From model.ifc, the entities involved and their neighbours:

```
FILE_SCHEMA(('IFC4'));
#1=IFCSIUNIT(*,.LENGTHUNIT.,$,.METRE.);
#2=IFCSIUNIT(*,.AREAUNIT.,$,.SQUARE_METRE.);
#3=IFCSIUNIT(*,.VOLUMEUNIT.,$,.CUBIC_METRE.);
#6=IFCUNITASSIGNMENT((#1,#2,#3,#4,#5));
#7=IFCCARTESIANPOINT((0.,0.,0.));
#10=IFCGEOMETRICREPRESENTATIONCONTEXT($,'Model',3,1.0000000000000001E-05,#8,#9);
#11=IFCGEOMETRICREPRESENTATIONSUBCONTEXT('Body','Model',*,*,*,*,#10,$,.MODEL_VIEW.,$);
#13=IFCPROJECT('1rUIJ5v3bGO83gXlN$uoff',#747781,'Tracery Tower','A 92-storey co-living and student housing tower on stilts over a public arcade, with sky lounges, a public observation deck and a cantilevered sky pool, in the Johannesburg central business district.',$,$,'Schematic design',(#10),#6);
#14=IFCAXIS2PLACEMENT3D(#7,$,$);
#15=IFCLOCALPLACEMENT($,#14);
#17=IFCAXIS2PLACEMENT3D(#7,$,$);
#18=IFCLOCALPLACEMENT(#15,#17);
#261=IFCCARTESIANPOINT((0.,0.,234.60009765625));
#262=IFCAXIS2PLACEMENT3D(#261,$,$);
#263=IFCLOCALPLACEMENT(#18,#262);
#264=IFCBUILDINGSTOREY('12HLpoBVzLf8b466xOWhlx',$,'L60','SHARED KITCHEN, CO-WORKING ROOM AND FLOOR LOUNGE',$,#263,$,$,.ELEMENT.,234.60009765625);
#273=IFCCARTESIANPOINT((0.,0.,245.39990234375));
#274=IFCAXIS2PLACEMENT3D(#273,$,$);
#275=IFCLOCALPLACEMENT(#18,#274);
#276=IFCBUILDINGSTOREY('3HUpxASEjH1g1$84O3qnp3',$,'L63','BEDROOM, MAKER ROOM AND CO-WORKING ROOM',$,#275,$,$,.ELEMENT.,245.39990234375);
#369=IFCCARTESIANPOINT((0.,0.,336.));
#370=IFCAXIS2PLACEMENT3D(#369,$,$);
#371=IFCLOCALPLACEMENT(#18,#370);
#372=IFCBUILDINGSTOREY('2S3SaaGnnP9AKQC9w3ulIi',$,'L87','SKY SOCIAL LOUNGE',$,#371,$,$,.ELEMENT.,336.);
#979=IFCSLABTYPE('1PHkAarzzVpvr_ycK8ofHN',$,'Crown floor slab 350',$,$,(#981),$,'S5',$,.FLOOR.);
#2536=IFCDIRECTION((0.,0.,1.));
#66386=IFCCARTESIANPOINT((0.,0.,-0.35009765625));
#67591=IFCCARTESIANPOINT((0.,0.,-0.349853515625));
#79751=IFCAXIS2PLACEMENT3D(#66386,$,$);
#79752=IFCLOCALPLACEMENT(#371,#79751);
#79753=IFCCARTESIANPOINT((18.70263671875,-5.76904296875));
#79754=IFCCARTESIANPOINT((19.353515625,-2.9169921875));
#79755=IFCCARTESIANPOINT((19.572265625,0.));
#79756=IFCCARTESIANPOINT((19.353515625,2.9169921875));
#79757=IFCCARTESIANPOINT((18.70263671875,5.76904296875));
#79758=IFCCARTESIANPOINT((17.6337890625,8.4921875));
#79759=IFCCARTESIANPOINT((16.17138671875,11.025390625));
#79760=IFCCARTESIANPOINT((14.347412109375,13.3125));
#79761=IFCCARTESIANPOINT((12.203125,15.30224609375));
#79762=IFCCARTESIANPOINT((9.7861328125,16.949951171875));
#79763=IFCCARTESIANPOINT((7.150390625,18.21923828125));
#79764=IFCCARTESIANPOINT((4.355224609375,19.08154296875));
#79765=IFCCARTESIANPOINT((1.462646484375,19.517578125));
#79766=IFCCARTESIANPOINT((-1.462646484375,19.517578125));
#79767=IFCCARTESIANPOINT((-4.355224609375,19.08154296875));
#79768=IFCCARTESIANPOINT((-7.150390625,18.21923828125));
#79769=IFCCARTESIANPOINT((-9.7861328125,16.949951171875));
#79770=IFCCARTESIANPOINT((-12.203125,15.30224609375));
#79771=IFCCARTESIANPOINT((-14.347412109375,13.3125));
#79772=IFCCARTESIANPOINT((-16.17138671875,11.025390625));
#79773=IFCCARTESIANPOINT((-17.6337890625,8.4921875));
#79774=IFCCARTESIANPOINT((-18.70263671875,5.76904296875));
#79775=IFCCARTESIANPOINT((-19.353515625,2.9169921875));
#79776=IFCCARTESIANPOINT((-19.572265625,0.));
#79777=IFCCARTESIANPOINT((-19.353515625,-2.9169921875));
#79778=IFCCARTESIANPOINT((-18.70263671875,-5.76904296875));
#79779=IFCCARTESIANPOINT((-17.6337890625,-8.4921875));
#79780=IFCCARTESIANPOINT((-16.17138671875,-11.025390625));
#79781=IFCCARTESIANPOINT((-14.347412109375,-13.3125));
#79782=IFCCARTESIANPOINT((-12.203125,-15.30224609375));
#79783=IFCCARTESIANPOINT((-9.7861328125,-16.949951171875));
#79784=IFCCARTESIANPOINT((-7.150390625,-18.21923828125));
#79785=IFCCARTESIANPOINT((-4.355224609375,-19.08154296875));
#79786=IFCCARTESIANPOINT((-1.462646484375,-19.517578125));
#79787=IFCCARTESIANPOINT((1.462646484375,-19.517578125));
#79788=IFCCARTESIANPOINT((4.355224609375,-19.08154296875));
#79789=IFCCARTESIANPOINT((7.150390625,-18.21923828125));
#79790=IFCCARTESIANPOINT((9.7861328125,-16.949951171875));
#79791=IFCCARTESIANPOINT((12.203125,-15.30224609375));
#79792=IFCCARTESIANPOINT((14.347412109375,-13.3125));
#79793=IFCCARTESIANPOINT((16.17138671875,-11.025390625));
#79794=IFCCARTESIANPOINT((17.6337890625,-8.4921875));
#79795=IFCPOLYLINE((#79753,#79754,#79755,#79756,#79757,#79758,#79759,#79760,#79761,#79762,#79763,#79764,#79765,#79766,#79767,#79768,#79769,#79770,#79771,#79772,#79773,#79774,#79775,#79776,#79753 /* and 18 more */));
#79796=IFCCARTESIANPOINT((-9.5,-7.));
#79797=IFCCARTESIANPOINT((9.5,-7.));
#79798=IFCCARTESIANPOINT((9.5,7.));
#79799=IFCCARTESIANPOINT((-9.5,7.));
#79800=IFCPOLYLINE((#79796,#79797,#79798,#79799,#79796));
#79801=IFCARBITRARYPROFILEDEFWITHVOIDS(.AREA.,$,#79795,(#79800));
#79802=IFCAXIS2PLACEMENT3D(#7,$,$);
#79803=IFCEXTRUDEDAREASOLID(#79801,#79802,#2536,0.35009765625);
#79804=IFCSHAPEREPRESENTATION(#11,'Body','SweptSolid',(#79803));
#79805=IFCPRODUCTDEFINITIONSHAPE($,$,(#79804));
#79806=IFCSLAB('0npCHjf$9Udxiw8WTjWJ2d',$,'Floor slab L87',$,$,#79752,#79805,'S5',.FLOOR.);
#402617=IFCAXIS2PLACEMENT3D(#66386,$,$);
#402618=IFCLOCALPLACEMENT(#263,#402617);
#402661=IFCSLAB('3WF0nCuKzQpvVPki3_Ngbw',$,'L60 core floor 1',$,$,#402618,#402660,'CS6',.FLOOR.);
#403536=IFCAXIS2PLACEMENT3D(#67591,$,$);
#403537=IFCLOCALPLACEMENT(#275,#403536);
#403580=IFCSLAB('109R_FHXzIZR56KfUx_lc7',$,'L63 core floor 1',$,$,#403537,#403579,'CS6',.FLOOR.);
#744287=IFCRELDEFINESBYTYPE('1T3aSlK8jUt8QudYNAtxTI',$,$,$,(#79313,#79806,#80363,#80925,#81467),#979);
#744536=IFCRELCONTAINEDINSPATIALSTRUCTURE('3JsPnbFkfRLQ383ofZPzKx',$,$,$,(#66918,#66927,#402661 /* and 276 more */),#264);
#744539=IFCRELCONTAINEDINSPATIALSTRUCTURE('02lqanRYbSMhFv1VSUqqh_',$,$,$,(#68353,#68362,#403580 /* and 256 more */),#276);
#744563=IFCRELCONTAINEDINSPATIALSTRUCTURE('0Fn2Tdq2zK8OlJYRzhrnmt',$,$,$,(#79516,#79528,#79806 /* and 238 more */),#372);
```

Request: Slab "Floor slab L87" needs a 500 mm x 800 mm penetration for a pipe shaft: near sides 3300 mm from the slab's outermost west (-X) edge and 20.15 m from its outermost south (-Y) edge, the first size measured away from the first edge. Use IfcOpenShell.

```python
import numpy as np
import ifcopenshell
import ifcopenshell.api.feature
import ifcopenshell.api.geometry
import ifcopenshell.api.root
import ifcopenshell.geom
import ifcopenshell.util.placement
import ifcopenshell.util.representation
import ifcopenshell.util.shape
import ifcopenshell.util.unit

model = ifcopenshell.open("model.ifc")
unit_scale = ifcopenshell.util.unit.calculate_unit_scale(model)
settings = ifcopenshell.geom.settings()


def volume(element):
    """Net volume in cubic metres, openings subtracted."""
    shape = ifcopenshell.geom.create_shape(settings, element)
    return ifcopenshell.util.shape.get_volume(shape.geometry)


slab = model.by_id(79806)
before = volume(slab)

# Extent in the slab's own axes, in metres. The edges named are its -X and -Y sides.
slab_shape = ifcopenshell.geom.create_shape(settings, slab)
vertices = ifcopenshell.util.shape.get_vertices(slab_shape.geometry)
x_min, y_min, bottom = vertices.min(axis=0)
top = vertices[:, 2].max()

opening = ifcopenshell.api.root.create_entity(model, ifc_class="IfcOpeningElement", name="Pipe shaft opening", predefined_type="OPENING")
context = ifcopenshell.util.representation.get_context(model, "Model", "Body", "MODEL_VIEW")
width, depth = 0.5, 0.8
outline = [(0.0, 0.0), (width, 0.0), (width, depth), (0.0, depth), (0.0, 0.0)]
# Overshoot both faces by 50 mm so the cut is clean.
shape = ifcopenshell.api.geometry.add_slab_representation(
    model, context=context, depth=top - bottom + 0.1, polyline=outline
)
ifcopenshell.api.geometry.assign_representation(model, product=opening, representation=shape)

matrix = ifcopenshell.util.placement.get_local_placement(slab.ObjectPlacement)
matrix[:, 3] = matrix @ np.append(np.array([x_min + 3.3, y_min + 20.15, bottom - 0.05]) / unit_scale, 1.0)
ifcopenshell.api.geometry.edit_object_placement(model, product=opening, matrix=matrix, is_si=False)
ifcopenshell.api.feature.add_feature(model, feature=opening, element=slab)

after = volume(slab)

print(f"slab volume {before:.3f} -> {after:.3f} m3")

model.write("model_rev.ifc")
```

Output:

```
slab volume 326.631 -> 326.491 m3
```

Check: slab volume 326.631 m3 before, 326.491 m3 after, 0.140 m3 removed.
